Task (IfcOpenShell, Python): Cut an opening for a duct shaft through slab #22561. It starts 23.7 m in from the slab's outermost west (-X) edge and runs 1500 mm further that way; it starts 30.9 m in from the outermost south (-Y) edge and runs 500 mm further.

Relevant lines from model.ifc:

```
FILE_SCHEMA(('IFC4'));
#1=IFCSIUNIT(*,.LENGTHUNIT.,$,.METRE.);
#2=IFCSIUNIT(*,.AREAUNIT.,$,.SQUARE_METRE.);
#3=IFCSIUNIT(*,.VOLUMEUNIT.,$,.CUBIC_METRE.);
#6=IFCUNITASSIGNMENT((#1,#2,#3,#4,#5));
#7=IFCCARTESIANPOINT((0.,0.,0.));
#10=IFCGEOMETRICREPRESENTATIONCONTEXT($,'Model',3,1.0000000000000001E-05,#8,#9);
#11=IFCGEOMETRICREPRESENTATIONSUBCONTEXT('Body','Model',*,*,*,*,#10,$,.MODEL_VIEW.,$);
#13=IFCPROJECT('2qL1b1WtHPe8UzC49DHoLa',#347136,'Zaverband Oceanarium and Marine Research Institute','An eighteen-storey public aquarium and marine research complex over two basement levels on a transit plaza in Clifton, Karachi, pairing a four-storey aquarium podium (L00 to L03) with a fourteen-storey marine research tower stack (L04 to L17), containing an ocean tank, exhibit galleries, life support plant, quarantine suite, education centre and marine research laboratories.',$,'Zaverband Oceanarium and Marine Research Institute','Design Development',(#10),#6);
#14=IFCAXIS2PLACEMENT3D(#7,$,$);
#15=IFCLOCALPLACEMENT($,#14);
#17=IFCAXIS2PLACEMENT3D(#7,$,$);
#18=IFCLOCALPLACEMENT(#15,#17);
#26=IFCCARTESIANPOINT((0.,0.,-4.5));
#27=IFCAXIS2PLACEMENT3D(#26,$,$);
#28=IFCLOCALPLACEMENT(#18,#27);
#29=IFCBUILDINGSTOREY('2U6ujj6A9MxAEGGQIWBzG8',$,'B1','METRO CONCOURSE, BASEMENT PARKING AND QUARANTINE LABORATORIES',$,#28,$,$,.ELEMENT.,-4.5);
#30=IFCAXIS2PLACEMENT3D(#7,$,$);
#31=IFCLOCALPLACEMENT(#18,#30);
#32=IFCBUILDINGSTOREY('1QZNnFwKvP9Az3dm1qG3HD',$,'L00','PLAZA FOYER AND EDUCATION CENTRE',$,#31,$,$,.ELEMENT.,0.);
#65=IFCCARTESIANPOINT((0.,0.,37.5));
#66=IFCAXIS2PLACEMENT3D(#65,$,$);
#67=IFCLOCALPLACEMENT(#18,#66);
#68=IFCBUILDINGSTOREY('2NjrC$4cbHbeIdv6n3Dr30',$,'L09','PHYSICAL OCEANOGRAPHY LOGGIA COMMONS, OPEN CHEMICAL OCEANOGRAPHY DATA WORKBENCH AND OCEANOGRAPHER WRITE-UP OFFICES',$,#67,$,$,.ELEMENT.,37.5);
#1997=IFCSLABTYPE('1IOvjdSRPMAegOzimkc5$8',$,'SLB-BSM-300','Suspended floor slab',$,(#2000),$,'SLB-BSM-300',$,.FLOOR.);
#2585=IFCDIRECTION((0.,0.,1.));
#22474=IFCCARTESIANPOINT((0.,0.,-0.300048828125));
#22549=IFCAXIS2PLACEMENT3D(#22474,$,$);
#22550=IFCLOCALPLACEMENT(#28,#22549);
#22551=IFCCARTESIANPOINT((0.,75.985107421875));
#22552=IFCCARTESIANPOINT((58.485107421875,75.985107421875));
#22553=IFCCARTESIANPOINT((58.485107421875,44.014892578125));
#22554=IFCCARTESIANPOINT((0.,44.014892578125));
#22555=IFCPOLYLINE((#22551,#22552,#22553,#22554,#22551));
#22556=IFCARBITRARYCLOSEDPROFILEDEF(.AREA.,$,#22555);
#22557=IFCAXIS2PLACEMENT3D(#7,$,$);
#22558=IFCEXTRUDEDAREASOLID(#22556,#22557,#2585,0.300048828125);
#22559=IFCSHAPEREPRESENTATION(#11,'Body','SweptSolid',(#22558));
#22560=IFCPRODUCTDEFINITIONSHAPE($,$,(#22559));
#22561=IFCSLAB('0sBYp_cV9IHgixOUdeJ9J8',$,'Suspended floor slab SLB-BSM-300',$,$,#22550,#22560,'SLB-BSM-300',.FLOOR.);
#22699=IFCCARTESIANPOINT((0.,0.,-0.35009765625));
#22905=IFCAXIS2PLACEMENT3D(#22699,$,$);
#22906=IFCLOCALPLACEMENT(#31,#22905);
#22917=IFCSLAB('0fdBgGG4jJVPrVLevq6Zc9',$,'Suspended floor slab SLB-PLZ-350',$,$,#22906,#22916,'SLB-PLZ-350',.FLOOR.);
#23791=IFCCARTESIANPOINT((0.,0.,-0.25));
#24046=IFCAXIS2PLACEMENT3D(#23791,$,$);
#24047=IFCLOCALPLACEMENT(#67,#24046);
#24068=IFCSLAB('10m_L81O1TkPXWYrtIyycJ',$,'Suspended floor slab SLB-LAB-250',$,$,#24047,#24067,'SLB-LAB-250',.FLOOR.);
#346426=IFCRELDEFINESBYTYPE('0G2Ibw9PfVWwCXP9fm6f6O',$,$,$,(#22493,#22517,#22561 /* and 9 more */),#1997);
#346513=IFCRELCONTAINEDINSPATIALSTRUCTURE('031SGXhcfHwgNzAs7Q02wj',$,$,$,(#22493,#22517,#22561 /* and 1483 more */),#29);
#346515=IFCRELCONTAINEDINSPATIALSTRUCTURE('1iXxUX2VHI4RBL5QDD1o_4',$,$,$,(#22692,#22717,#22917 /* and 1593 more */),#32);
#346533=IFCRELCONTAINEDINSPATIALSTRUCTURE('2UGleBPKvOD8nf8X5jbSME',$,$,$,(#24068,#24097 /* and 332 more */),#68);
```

```python
import numpy as np
import ifcopenshell
import ifcopenshell.api.feature
import ifcopenshell.api.geometry
import ifcopenshell.api.root
import ifcopenshell.geom
import ifcopenshell.util.placement
import ifcopenshell.util.representation
import ifcopenshell.util.shape
import ifcopenshell.util.unit

model = ifcopenshell.open("model.ifc")
unit_scale = ifcopenshell.util.unit.calculate_unit_scale(model)
settings = ifcopenshell.geom.settings()


def volume(element):
    """Net volume in cubic metres, openings subtracted."""
    shape = ifcopenshell.geom.create_shape(settings, element)
    return ifcopenshell.util.shape.get_volume(shape.geometry)


slab = model.by_guid("0sBYp_cV9IHgixOUdeJ9J8")
before = volume(slab)

# Extent in the slab's own axes, in metres. The edges named are its -X and -Y sides.
slab_shape = ifcopenshell.geom.create_shape(settings, slab)
vertices = ifcopenshell.util.shape.get_vertices(slab_shape.geometry)
x_min, y_min, bottom = vertices.min(axis=0)
top = vertices[:, 2].max()

opening = ifcopenshell.api.root.create_entity(model, ifc_class="IfcOpeningElement", name="Duct shaft opening", predefined_type="OPENING")
context = ifcopenshell.util.representation.get_context(model, "Model", "Body", "MODEL_VIEW")
width, depth = 1.5, 0.5
outline = [(0.0, 0.0), (width, 0.0), (width, depth), (0.0, depth), (0.0, 0.0)]
# Overshoot both faces by 50 mm so the cut is clean.
shape = ifcopenshell.api.geometry.add_slab_representation(
    model, context=context, depth=top - bottom + 0.1, polyline=outline
)
ifcopenshell.api.geometry.assign_representation(model, product=opening, representation=shape)

matrix = ifcopenshell.util.placement.get_local_placement(slab.ObjectPlacement)
matrix[:, 3] = matrix @ np.append(np.array([x_min + 23.7, y_min + 30.9, bottom - 0.05]) / unit_scale, 1.0)
ifcopenshell.api.geometry.edit_object_placement(model, product=opening, matrix=matrix, is_si=False)
ifcopenshell.api.feature.add_feature(model, feature=opening, element=slab)

after = volume(slab)

print(f"slab volume {before:.3f} -> {after:.3f} m3")

model.write("model_rev.ifc")
```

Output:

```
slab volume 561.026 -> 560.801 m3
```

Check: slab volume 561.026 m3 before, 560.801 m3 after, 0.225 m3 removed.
